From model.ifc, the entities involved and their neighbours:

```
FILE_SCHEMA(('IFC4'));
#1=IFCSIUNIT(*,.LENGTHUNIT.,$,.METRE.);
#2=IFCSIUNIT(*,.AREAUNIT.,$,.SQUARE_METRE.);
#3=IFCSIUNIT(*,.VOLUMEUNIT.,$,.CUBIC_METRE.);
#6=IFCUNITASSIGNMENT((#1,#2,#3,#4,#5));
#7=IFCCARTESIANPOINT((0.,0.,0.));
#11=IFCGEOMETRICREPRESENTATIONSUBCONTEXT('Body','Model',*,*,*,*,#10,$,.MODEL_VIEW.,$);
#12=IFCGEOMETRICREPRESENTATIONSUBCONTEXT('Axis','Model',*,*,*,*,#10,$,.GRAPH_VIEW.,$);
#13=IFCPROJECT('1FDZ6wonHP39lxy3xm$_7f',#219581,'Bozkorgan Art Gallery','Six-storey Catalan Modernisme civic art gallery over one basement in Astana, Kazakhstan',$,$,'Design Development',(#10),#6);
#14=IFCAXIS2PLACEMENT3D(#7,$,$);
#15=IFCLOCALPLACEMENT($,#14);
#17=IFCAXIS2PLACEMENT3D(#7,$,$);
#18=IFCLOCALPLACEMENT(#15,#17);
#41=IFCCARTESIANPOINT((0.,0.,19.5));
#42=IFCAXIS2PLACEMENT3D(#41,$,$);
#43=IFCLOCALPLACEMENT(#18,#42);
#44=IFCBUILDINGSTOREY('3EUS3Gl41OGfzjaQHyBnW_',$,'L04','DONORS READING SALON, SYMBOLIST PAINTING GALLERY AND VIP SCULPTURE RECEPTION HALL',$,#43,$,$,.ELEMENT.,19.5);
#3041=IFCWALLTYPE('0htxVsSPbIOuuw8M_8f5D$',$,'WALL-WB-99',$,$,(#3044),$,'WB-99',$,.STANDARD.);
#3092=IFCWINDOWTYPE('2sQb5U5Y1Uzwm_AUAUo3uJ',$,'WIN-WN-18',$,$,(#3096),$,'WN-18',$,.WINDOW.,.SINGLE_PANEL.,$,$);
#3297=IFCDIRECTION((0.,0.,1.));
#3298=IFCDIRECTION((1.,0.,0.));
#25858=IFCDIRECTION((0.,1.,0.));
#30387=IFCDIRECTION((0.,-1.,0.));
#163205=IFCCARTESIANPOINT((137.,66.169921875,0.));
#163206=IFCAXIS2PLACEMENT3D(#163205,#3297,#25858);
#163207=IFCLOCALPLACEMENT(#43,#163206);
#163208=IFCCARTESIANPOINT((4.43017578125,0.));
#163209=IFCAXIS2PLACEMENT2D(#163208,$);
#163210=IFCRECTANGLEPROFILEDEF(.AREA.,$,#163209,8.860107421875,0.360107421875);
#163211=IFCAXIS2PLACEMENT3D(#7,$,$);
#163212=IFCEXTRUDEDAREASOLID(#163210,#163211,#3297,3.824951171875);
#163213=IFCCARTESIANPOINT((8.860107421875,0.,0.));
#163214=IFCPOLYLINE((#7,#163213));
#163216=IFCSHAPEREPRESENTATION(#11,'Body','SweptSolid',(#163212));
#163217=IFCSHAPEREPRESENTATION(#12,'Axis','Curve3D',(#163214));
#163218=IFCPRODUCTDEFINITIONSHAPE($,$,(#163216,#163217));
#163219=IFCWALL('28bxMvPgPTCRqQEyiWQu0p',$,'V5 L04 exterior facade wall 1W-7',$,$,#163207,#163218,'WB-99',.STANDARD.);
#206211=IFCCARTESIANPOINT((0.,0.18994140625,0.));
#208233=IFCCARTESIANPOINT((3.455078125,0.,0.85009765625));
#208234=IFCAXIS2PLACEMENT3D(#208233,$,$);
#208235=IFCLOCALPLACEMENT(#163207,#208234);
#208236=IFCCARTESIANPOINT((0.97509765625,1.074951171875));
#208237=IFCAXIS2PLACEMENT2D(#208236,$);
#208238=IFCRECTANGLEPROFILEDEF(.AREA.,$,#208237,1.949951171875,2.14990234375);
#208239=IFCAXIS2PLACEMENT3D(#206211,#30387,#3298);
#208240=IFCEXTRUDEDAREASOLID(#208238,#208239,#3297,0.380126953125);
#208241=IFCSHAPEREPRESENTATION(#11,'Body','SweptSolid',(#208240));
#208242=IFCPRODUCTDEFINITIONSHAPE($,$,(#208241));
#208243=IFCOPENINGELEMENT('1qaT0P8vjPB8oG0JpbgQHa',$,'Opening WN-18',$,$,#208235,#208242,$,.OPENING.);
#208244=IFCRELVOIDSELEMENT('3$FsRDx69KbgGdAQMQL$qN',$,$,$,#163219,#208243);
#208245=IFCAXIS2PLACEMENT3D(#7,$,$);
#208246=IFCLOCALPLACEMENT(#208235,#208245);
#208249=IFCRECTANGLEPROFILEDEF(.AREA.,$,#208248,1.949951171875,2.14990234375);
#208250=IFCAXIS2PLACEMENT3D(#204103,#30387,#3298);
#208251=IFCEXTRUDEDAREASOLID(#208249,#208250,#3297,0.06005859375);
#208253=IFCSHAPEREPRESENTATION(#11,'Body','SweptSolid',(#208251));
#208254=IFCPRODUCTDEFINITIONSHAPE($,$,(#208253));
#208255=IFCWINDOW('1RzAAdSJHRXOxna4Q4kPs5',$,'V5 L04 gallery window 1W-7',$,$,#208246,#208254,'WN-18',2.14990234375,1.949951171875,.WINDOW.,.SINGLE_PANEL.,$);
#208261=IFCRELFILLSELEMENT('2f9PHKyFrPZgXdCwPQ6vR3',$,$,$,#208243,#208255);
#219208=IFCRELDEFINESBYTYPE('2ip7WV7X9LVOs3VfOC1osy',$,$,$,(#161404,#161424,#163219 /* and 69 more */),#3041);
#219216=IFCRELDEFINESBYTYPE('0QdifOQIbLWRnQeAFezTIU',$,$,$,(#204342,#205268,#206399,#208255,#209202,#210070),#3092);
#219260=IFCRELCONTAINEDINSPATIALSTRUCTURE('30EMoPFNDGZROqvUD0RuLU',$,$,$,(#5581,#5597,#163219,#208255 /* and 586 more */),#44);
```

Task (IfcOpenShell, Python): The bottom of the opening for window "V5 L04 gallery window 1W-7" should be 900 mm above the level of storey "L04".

```python
import numpy as np
import ifcopenshell
import ifcopenshell.api.geometry
import ifcopenshell.geom
import ifcopenshell.util.element
import ifcopenshell.util.placement
import ifcopenshell.util.shape
import ifcopenshell.util.unit

model = ifcopenshell.open("model.ifc")
unit_scale = ifcopenshell.util.unit.calculate_unit_scale(model)

window = model.by_guid("1RzAAdSJHRXOxna4Q4kPs5")
opening = window.FillsVoids[0].RelatingOpeningElement
storey = ifcopenshell.util.element.get_container(window, ifc_class="IfcBuildingStorey")
level = ifcopenshell.util.placement.get_local_placement(storey.ObjectPlacement)[2, 3]

# The opening's origin need not be at the sill, so measure its lowest point.
shape = ifcopenshell.geom.create_shape(ifcopenshell.geom.settings(), opening)
bottom = ifcopenshell.util.shape.get_shape_bottom_elevation(shape, shape.geometry) / unit_scale
dz = level + 0.9 / unit_scale - bottom

shift = np.array([0.0, 0.0, dz])
# The window is placed relative to its opening, so it follows when the opening moves.
matrix = ifcopenshell.util.placement.get_local_placement(opening.ObjectPlacement)
matrix[:3, 3] += shift
ifcopenshell.api.geometry.edit_object_placement(
    model, product=opening, matrix=matrix, is_si=False, should_transform_children=True
)

print(f"moved by {dz * unit_scale:+.3f} m")

model.write("model-out.ifc")
```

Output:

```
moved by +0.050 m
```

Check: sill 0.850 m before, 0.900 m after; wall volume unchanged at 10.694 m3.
